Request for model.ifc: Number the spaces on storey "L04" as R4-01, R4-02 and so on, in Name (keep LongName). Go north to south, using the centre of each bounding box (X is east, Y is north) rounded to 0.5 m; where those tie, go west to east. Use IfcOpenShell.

First a look at what the model holds.

```python
import ifcopenshell
import ifcopenshell.util.element
import ifcopenshell.util.placement

model = ifcopenshell.open("model.ifc")
print(model.schema)
storey = next(s for s in model.by_type("IfcBuildingStorey") if s.Name == "L04")
spaces = [e for e in ifcopenshell.util.element.get_decomposition(storey) if e.is_a("IfcSpace")]
for e in sorted(spaces, key=lambda e: e.id()):
    origin = ifcopenshell.util.placement.get_local_placement(e.ObjectPlacement)[:3, 3]
    print(e.id(), e.Name, e.LongName, origin.round(2) + 0.0, sep=" | ")
```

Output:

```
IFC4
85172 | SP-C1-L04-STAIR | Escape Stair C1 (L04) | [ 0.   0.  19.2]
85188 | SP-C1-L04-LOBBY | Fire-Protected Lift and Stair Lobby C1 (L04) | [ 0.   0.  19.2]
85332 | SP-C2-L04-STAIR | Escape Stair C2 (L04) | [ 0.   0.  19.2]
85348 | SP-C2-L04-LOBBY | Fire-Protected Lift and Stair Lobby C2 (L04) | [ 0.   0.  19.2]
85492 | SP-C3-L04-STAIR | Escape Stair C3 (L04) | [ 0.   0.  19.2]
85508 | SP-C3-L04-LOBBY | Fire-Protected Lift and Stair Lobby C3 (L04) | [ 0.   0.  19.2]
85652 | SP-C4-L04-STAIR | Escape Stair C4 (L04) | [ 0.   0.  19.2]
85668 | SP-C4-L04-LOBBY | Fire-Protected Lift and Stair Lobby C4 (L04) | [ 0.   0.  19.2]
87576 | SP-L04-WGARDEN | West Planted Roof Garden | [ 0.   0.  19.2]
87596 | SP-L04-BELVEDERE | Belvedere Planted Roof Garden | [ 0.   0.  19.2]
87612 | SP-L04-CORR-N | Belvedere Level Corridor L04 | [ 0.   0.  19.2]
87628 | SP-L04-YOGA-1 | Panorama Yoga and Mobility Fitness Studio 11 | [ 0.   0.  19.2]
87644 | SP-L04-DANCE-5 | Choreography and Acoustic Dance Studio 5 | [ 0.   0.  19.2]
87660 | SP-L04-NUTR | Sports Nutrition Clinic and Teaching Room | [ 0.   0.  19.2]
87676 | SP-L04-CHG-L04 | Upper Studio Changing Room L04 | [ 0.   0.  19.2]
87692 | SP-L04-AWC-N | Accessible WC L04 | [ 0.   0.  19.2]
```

```python
import ifcopenshell
import ifcopenshell.geom
import ifcopenshell.util.element
import ifcopenshell.util.shape

model = ifcopenshell.open("model.ifc")
settings = ifcopenshell.geom.settings()
settings.set("use-world-coords", True)


def centre(element):
    shape = ifcopenshell.geom.create_shape(settings, element)
    return ifcopenshell.util.shape.get_bbox_centroid(shape.geometry)


storey = next(s for s in model.by_type("IfcBuildingStorey") if s.Name == "L04")
spaces = [e for e in ifcopenshell.util.element.get_decomposition(storey) if e.is_a("IfcSpace")]

# Insertion points can sit at a corner or the storey origin, so sort by the geometry (in metres).
centres = {e: centre(e) for e in spaces}
spaces.sort(key=lambda e: (-round(centres[e][1] / 0.5), centres[e][0]))

for i, e in enumerate(spaces, start=1):
    number = f"R4-{i:02d}"
    e.Name = number
    print(e.id(), number)

model.write("model_edited.ifc")
```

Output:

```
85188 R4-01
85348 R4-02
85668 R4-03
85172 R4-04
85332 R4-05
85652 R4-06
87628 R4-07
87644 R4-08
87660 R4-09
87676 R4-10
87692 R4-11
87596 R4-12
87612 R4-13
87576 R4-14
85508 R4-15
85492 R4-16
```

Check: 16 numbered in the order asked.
